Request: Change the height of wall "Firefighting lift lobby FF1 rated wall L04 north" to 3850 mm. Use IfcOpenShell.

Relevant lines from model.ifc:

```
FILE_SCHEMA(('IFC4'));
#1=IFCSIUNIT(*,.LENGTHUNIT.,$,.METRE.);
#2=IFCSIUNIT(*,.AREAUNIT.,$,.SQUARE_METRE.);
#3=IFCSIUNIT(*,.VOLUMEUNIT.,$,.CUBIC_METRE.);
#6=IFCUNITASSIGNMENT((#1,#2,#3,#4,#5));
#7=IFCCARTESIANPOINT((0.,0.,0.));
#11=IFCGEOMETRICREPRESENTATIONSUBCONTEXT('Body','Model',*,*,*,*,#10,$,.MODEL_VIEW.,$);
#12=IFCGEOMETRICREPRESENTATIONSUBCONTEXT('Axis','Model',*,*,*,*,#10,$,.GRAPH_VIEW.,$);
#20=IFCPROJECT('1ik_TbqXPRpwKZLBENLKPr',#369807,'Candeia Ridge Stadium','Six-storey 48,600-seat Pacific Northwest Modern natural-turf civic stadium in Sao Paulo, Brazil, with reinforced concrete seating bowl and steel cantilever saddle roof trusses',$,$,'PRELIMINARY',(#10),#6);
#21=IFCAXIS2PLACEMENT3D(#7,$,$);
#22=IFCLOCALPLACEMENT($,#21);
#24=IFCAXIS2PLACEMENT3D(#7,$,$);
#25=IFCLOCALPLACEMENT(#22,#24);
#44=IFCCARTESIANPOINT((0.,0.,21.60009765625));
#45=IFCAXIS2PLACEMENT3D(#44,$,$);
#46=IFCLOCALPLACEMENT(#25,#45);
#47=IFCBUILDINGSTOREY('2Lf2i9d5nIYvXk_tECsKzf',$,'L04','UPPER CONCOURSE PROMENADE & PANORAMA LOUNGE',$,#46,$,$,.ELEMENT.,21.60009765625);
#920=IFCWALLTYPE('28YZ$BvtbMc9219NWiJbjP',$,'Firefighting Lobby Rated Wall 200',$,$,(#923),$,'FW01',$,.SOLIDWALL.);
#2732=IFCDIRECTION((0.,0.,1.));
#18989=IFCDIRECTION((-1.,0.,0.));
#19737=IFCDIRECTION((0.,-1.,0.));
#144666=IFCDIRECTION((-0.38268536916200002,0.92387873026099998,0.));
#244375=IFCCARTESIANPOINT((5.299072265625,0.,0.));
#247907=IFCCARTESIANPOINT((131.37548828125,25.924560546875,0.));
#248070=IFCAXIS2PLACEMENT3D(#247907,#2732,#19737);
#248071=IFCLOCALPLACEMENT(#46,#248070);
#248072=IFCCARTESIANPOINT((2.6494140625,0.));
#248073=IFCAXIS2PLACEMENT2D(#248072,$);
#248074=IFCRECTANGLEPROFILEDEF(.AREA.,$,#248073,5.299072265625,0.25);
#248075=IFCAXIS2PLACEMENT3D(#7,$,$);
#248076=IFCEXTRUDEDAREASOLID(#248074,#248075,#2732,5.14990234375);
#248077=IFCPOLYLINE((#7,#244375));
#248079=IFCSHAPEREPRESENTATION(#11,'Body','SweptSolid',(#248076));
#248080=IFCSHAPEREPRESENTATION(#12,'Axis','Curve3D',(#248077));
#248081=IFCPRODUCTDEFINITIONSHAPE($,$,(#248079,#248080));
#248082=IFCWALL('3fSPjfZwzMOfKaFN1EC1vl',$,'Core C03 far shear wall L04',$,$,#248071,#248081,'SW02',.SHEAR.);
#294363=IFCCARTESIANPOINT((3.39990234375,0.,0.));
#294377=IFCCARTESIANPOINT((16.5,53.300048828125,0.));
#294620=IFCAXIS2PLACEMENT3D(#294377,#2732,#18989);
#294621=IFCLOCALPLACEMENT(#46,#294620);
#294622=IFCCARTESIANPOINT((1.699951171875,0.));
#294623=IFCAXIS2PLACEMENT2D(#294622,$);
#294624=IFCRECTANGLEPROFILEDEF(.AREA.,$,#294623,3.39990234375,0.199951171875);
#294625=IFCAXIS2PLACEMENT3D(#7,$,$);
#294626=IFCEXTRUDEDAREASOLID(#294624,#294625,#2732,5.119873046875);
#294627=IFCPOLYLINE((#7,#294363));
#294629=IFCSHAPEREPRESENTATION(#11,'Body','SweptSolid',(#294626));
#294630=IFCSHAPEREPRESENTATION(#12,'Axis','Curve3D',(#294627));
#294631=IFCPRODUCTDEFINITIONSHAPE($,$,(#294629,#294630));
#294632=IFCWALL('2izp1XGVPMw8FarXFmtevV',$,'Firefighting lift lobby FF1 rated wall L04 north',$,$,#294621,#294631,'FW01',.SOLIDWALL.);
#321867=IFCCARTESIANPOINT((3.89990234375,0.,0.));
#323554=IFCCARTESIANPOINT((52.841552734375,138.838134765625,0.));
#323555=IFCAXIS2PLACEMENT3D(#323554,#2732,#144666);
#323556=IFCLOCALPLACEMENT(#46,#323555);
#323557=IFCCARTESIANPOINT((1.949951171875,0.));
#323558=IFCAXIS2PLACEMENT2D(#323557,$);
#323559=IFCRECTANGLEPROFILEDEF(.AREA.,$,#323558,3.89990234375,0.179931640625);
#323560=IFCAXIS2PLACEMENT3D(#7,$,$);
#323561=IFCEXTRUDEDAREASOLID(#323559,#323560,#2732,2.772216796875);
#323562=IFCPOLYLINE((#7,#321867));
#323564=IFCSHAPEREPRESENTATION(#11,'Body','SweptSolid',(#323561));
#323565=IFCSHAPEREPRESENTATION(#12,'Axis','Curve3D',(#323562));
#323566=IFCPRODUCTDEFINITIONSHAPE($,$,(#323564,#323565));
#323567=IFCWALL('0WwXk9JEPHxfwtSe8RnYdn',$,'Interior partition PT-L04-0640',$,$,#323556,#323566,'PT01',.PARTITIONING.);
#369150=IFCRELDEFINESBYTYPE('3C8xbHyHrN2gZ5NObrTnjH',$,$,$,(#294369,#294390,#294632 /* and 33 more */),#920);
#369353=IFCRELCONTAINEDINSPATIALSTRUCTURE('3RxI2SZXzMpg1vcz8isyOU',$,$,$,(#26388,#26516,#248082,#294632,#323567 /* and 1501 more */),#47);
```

```python
import ifcopenshell
import ifcopenshell.geom
import ifcopenshell.util.representation
import ifcopenshell.util.shape

model = ifcopenshell.open("model.ifc")
settings = ifcopenshell.geom.settings()


def volume(element):
    """Net volume in cubic metres, openings subtracted."""
    shape = ifcopenshell.geom.create_shape(settings, element)
    return ifcopenshell.util.shape.get_volume(shape.geometry)


wall = model.by_guid("2izp1XGVPMw8FarXFmtevV")
before = volume(wall)

body = ifcopenshell.util.representation.get_representation(wall, "Model", "Body")
solid = body.Items[0]
old_height = solid.Depth
solid.Depth = 3.85
after = volume(wall)

print(f"height {old_height:g} -> {solid.Depth:g}, volume {before:.3f} -> {after:.3f} m3")

model.write("model-out.ifc")
```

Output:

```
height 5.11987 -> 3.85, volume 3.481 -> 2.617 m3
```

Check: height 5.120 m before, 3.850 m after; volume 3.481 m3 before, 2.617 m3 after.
